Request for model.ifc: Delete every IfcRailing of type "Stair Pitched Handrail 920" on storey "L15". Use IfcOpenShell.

First a look at what the model holds.

```python
import ifcopenshell
import ifcopenshell.util.element

model = ifcopenshell.open("model.ifc")
print(model.schema)
storey = next(s for s in model.by_type("IfcBuildingStorey") if s.Name == "L15")
railings = [e for e in ifcopenshell.util.element.get_decomposition(storey) if e.is_a("IfcRailing")]
seen = {}
for e in railings:
    element_type = ifcopenshell.util.element.get_type(e)
    name = element_type.Name if element_type not in (None, e) else None
    seen[name] = seen.get(name, 0) + 1
for name, count in sorted(seen.items(), key=str):
    print(count, "x", name)
```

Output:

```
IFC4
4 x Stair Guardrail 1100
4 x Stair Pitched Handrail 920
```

```python
import ifcopenshell
import ifcopenshell.api.root
import ifcopenshell.util.element

model = ifcopenshell.open("model.ifc")

storey = next(s for s in model.by_type("IfcBuildingStorey") if s.Name == "L15")
railings = [e for e in ifcopenshell.util.element.get_decomposition(storey) if e.is_a("IfcRailing")]
targets = [e for e in railings if (t := ifcopenshell.util.element.get_type(e)) not in (None, e) and t.Name == "Stair Pitched Handrail 920"]

for e in targets:
    ifcopenshell.api.root.remove_product(model, product=e)
print(len(targets), "removed")

model.write("model-out.ifc")
```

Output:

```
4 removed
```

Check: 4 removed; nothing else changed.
